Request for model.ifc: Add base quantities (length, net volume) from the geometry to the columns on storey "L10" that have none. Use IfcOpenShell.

First a look at what the model holds.

```python
import ifcopenshell
import ifcopenshell.util.element
import ifcopenshell.util.unit

model = ifcopenshell.open("model.ifc")
print(model.schema)
for unit_type in ("LENGTHUNIT", "AREAUNIT", "VOLUMEUNIT"):
    print(unit_type, ifcopenshell.util.unit.calculate_unit_scale(model, unit_type))
storey = next(s for s in model.by_type("IfcBuildingStorey") if s.Name == "L10")
columns = [e for e in ifcopenshell.util.element.get_decomposition(storey) if e.is_a("IfcColumn")]
for e in sorted(columns, key=lambda e: e.id()):
    print(e.id(), e.is_a(), e.Name, list(ifcopenshell.util.element.get_psets(e, qtos_only=True)), sep=" | ")
```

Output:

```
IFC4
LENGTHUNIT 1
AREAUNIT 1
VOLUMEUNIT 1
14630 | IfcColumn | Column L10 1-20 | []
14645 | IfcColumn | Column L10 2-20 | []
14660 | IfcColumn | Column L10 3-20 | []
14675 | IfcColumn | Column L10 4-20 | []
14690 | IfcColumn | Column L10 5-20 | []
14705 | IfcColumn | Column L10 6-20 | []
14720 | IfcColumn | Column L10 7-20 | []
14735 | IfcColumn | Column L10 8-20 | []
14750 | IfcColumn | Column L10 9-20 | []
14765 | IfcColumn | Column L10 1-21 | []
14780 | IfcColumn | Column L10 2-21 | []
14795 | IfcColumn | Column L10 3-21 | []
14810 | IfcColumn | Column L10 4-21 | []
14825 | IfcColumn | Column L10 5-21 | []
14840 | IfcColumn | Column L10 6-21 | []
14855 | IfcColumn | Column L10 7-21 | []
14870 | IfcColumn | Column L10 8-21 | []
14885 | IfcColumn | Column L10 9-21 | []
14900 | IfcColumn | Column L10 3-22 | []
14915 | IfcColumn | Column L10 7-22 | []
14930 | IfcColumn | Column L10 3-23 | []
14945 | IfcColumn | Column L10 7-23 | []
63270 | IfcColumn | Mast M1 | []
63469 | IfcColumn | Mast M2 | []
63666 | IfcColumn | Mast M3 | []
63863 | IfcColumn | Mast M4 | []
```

```python
import ifcopenshell
import ifcopenshell.api.pset
import ifcopenshell.geom
import ifcopenshell.util.element
import ifcopenshell.util.shape
import ifcopenshell.util.unit

model = ifcopenshell.open("model.ifc")
unit_scale = ifcopenshell.util.unit.calculate_unit_scale(model)
volume_scale = ifcopenshell.util.unit.calculate_unit_scale(model, "VOLUMEUNIT")
settings = ifcopenshell.geom.settings()

storey = next(s for s in model.by_type("IfcBuildingStorey") if s.Name == "L10")
columns = [e for e in ifcopenshell.util.element.get_decomposition(storey) if e.is_a("IfcColumn")]

for e in sorted(columns, key=lambda e: e.id()):
    if ifcopenshell.util.element.get_psets(e, qtos_only=True, should_inherit=False):
        continue
    # Geometry comes back in metres, in the element's own axes.
    shape = ifcopenshell.geom.create_shape(settings, e)
    values = {
        "Length": ifcopenshell.util.shape.get_z(shape.geometry) / unit_scale,
        "NetVolume": ifcopenshell.util.shape.get_volume(shape.geometry) / volume_scale,
    }
    qto = ifcopenshell.api.pset.add_qto(model, product=e, name="Qto_ColumnBaseQuantities")
    ifcopenshell.api.pset.edit_qto(model, qto=qto, properties=values)
    print(e.id(), {k: round(v, 3) for k, v in values.items()})

model.write("model_edited.ifc")
```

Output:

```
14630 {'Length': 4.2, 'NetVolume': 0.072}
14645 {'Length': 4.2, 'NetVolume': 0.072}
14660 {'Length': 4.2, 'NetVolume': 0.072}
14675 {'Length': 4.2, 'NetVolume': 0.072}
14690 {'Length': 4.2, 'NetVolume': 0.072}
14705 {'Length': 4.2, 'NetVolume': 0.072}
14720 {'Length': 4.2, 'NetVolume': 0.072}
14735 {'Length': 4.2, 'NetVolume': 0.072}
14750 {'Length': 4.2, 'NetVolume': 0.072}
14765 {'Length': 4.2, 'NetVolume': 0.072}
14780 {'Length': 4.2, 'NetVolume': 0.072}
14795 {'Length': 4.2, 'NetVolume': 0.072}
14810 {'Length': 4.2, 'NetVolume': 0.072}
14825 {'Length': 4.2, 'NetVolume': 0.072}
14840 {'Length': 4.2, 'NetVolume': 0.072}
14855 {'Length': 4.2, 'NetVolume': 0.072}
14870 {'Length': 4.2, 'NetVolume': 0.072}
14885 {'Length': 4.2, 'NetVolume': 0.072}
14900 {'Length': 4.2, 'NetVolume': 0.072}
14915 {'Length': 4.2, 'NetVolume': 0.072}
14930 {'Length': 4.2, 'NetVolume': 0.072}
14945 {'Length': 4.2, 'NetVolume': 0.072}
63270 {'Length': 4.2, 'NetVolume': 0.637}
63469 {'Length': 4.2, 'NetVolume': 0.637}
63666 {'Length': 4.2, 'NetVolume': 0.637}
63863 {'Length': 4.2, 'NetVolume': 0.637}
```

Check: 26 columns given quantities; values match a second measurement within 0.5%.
